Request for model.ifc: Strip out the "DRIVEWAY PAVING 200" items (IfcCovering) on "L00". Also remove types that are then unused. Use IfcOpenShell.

First a look at what the model holds.

```python
import ifcopenshell
import ifcopenshell.util.element

model = ifcopenshell.open("model.ifc")
print(model.schema)
storey = next(s for s in model.by_type("IfcBuildingStorey") if s.Name == "L00")
coverings = [e for e in ifcopenshell.util.element.get_decomposition(storey) if e.is_a("IfcCovering")]
seen = {}
for e in coverings:
    element_type = ifcopenshell.util.element.get_type(e)
    name = element_type.Name if element_type not in (None, e) else None
    seen[name] = seen.get(name, 0) + 1
for name, count in sorted(seen.items(), key=str):
    print(count, "x", name)
```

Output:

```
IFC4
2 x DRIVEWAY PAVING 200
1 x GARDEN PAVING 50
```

```python
import ifcopenshell
import ifcopenshell.api.root
import ifcopenshell.util.element

model = ifcopenshell.open("model.ifc")

storey = next(s for s in model.by_type("IfcBuildingStorey") if s.Name == "L00")
coverings = [e for e in ifcopenshell.util.element.get_decomposition(storey) if e.is_a("IfcCovering")]
targets = [e for e in coverings if (t := ifcopenshell.util.element.get_type(e)) not in (None, e) and t.Name == "DRIVEWAY PAVING 200"]
types = {ifcopenshell.util.element.get_type(e) for e in targets} - {None, *targets}

for e in targets:
    ifcopenshell.api.root.remove_product(model, product=e)
print(len(targets), "removed")

unused = [t for t in types if not ifcopenshell.util.element.get_types(t)]
for t in unused:
    ifcopenshell.api.root.remove_product(model, product=t)
print(len(unused), "unused types removed")

model.write("model_rev.ifc")
```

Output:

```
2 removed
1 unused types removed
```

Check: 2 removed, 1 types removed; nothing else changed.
